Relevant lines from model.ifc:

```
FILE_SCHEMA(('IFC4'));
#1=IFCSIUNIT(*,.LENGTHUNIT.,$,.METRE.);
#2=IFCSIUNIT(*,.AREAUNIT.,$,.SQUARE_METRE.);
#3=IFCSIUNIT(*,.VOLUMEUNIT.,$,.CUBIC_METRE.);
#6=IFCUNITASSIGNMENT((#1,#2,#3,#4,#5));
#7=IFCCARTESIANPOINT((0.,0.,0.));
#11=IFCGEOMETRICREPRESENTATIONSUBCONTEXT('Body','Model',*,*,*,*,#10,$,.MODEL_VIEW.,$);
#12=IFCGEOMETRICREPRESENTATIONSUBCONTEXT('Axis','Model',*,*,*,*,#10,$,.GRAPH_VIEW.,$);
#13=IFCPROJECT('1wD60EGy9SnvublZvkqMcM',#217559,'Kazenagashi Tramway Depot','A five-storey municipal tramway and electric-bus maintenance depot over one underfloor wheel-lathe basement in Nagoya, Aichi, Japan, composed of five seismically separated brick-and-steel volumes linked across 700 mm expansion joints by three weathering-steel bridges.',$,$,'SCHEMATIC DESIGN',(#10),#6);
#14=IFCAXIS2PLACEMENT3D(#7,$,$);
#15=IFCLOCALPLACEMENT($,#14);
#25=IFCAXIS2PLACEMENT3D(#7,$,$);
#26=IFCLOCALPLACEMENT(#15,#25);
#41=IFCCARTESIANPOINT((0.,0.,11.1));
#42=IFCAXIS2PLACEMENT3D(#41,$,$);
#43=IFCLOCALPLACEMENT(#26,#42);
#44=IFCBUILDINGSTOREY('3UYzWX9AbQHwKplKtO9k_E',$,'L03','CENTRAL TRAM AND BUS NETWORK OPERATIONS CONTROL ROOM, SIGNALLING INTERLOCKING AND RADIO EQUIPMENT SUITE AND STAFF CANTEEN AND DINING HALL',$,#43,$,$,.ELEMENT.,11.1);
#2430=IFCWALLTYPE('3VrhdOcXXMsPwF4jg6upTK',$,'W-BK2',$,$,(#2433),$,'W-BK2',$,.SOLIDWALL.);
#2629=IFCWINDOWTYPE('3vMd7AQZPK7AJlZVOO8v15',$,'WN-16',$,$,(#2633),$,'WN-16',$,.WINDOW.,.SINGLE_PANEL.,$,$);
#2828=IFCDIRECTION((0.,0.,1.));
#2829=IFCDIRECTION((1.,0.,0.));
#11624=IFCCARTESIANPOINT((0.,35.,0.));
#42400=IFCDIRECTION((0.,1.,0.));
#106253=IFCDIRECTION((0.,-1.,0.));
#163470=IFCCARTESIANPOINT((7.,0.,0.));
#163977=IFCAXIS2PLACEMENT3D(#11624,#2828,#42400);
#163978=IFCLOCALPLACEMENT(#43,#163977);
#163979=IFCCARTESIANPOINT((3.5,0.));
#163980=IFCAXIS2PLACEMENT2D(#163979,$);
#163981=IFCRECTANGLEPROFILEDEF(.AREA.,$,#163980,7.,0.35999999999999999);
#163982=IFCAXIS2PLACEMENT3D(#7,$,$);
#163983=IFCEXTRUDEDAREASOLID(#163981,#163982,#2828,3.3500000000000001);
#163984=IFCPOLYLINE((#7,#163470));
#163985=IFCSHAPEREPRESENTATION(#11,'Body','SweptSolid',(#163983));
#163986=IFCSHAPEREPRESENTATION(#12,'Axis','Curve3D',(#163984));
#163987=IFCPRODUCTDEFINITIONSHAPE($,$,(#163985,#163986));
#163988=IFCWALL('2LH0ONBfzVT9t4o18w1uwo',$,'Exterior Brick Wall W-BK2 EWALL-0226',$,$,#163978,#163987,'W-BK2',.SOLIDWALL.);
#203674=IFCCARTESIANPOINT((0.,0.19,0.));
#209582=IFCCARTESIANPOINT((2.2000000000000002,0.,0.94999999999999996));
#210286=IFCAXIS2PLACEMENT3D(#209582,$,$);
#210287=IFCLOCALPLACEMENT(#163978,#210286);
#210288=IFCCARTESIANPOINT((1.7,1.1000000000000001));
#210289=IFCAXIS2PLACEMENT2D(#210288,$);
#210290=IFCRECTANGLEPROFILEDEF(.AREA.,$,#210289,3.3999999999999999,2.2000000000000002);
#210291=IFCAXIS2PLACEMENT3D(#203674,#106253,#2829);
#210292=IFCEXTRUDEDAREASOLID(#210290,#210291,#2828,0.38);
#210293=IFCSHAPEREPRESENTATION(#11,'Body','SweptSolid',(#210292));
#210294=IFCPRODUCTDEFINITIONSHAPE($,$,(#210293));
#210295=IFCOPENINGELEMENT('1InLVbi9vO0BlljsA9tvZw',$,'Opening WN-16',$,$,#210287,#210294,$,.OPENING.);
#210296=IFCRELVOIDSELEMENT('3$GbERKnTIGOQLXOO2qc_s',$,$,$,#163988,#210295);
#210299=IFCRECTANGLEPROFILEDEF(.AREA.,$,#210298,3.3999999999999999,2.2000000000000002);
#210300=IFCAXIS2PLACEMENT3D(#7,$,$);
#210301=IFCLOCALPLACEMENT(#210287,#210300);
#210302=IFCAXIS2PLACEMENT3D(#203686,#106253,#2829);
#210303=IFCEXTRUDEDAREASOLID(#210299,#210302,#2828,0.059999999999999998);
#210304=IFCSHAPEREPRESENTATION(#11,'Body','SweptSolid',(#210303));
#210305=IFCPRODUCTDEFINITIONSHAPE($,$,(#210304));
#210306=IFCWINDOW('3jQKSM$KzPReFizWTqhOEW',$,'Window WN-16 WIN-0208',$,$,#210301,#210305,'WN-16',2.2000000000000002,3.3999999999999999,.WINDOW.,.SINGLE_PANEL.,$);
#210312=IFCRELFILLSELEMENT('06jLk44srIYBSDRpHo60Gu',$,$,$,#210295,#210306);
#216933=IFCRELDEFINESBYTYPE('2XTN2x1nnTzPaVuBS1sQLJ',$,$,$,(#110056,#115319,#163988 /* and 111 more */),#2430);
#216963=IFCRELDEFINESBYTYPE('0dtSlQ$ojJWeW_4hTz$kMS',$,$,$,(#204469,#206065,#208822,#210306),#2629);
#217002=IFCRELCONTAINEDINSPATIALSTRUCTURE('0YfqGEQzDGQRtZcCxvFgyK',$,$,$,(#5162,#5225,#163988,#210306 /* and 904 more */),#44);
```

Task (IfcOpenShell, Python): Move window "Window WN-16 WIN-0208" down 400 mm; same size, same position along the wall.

```python
import numpy as np
import ifcopenshell
import ifcopenshell.api.geometry
import ifcopenshell.util.placement
import ifcopenshell.util.unit

model = ifcopenshell.open("model.ifc")
unit_scale = ifcopenshell.util.unit.calculate_unit_scale(model)

window = model.by_guid("3jQKSM$KzPReFizWTqhOEW")
opening = window.FillsVoids[0].RelatingOpeningElement
dz = -0.4 / unit_scale

shift = np.array([0.0, 0.0, dz])
# The window is placed relative to its opening, so it follows when the opening moves.
matrix = ifcopenshell.util.placement.get_local_placement(opening.ObjectPlacement)
matrix[:3, 3] += shift
ifcopenshell.api.geometry.edit_object_placement(
    model, product=opening, matrix=matrix, is_si=False, should_transform_children=True
)

print(f"moved by {dz * unit_scale:+.3f} m")

model.write("model-out.ifc")
```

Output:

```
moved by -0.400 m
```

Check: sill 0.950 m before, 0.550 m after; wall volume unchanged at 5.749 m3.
